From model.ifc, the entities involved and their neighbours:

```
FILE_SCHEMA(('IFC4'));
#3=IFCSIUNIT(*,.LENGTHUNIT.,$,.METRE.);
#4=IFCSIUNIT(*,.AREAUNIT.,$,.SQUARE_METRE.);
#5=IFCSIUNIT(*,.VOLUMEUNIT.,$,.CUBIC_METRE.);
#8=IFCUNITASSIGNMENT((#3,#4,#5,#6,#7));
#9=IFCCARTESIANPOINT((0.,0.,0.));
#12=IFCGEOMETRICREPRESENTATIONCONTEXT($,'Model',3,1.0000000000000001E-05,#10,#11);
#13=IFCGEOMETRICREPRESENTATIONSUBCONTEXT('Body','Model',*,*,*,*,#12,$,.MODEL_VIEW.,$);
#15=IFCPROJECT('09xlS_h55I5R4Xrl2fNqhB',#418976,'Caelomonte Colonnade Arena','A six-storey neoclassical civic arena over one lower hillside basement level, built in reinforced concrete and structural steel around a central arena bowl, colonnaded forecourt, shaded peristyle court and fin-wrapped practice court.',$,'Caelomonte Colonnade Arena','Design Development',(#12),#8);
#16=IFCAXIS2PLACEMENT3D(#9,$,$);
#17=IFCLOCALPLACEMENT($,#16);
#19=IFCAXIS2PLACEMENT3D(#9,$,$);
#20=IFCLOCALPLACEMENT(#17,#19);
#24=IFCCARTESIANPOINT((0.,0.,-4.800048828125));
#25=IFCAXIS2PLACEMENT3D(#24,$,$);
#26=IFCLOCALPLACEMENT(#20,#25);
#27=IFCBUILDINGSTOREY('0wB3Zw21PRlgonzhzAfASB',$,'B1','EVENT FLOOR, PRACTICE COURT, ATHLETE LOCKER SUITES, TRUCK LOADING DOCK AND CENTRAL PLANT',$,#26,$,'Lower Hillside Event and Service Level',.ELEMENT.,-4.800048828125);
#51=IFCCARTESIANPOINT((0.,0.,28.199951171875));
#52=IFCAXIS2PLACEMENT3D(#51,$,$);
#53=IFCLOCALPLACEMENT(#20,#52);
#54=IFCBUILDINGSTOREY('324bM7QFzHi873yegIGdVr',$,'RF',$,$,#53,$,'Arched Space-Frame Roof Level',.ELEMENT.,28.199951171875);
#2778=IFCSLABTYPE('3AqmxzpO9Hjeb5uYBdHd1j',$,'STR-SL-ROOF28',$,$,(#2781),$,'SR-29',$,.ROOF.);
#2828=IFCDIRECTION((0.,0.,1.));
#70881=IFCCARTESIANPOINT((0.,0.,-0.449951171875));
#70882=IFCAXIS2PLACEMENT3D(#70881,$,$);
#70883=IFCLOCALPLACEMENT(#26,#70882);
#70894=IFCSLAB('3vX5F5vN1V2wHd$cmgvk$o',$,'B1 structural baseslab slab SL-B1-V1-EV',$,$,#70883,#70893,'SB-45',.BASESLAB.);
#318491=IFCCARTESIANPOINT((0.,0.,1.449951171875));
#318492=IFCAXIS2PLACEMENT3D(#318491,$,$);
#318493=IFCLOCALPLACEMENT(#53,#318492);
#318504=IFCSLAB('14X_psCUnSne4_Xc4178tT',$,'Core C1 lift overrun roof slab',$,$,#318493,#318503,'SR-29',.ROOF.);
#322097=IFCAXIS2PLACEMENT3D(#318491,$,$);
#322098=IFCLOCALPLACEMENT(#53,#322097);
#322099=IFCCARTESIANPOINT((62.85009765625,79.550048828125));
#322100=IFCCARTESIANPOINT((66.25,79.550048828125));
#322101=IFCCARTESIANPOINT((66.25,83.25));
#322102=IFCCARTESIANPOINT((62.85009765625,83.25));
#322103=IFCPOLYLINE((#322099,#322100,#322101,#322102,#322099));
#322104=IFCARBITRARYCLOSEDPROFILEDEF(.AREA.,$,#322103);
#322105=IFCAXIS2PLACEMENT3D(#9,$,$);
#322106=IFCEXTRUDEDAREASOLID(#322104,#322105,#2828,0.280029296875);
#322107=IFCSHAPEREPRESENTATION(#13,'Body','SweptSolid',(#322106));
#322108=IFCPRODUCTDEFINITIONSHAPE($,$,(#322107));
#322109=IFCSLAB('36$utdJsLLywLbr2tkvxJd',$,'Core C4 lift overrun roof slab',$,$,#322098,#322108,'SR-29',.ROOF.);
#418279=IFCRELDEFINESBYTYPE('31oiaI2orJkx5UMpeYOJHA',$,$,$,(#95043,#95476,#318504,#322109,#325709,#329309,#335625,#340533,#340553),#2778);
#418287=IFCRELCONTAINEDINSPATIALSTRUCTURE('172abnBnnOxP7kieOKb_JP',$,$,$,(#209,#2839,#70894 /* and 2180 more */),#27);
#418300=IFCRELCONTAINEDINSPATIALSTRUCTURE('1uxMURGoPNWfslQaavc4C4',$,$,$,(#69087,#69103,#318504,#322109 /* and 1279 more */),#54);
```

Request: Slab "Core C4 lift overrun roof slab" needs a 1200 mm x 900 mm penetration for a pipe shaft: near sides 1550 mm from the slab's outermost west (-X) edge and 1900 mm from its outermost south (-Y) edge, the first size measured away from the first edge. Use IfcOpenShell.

```python
import numpy as np
import ifcopenshell
import ifcopenshell.api.feature
import ifcopenshell.api.geometry
import ifcopenshell.api.root
import ifcopenshell.geom
import ifcopenshell.util.placement
import ifcopenshell.util.representation
import ifcopenshell.util.shape
import ifcopenshell.util.unit

model = ifcopenshell.open("model.ifc")
unit_scale = ifcopenshell.util.unit.calculate_unit_scale(model)
settings = ifcopenshell.geom.settings()


def volume(element):
    """Net volume in cubic metres, openings subtracted."""
    shape = ifcopenshell.geom.create_shape(settings, element)
    return ifcopenshell.util.shape.get_volume(shape.geometry)


slab = model.by_guid("36$utdJsLLywLbr2tkvxJd")
before = volume(slab)

# Extent in the slab's own axes, in metres. The edges named are its -X and -Y sides.
slab_shape = ifcopenshell.geom.create_shape(settings, slab)
vertices = ifcopenshell.util.shape.get_vertices(slab_shape.geometry)
x_min, y_min, bottom = vertices.min(axis=0)
top = vertices[:, 2].max()

opening = ifcopenshell.api.root.create_entity(model, ifc_class="IfcOpeningElement", name="Pipe shaft opening", predefined_type="OPENING")
context = ifcopenshell.util.representation.get_context(model, "Model", "Body", "MODEL_VIEW")
width, depth = 1.2, 0.9
outline = [(0.0, 0.0), (width, 0.0), (width, depth), (0.0, depth), (0.0, 0.0)]
# Overshoot both faces by 50 mm so the cut is clean.
shape = ifcopenshell.api.geometry.add_slab_representation(
    model, context=context, depth=top - bottom + 0.1, polyline=outline
)
ifcopenshell.api.geometry.assign_representation(model, product=opening, representation=shape)

matrix = ifcopenshell.util.placement.get_local_placement(slab.ObjectPlacement)
matrix[:, 3] = matrix @ np.append(np.array([x_min + 1.55, y_min + 1.9, bottom - 0.05]) / unit_scale, 1.0)
ifcopenshell.api.geometry.edit_object_placement(model, product=opening, matrix=matrix, is_si=False)
ifcopenshell.api.feature.add_feature(model, feature=opening, element=slab)

after = volume(slab)

print(f"slab volume {before:.3f} -> {after:.3f} m3")

model.write("model_updated.ifc")
```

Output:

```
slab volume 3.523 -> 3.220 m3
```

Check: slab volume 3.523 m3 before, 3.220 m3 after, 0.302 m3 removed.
